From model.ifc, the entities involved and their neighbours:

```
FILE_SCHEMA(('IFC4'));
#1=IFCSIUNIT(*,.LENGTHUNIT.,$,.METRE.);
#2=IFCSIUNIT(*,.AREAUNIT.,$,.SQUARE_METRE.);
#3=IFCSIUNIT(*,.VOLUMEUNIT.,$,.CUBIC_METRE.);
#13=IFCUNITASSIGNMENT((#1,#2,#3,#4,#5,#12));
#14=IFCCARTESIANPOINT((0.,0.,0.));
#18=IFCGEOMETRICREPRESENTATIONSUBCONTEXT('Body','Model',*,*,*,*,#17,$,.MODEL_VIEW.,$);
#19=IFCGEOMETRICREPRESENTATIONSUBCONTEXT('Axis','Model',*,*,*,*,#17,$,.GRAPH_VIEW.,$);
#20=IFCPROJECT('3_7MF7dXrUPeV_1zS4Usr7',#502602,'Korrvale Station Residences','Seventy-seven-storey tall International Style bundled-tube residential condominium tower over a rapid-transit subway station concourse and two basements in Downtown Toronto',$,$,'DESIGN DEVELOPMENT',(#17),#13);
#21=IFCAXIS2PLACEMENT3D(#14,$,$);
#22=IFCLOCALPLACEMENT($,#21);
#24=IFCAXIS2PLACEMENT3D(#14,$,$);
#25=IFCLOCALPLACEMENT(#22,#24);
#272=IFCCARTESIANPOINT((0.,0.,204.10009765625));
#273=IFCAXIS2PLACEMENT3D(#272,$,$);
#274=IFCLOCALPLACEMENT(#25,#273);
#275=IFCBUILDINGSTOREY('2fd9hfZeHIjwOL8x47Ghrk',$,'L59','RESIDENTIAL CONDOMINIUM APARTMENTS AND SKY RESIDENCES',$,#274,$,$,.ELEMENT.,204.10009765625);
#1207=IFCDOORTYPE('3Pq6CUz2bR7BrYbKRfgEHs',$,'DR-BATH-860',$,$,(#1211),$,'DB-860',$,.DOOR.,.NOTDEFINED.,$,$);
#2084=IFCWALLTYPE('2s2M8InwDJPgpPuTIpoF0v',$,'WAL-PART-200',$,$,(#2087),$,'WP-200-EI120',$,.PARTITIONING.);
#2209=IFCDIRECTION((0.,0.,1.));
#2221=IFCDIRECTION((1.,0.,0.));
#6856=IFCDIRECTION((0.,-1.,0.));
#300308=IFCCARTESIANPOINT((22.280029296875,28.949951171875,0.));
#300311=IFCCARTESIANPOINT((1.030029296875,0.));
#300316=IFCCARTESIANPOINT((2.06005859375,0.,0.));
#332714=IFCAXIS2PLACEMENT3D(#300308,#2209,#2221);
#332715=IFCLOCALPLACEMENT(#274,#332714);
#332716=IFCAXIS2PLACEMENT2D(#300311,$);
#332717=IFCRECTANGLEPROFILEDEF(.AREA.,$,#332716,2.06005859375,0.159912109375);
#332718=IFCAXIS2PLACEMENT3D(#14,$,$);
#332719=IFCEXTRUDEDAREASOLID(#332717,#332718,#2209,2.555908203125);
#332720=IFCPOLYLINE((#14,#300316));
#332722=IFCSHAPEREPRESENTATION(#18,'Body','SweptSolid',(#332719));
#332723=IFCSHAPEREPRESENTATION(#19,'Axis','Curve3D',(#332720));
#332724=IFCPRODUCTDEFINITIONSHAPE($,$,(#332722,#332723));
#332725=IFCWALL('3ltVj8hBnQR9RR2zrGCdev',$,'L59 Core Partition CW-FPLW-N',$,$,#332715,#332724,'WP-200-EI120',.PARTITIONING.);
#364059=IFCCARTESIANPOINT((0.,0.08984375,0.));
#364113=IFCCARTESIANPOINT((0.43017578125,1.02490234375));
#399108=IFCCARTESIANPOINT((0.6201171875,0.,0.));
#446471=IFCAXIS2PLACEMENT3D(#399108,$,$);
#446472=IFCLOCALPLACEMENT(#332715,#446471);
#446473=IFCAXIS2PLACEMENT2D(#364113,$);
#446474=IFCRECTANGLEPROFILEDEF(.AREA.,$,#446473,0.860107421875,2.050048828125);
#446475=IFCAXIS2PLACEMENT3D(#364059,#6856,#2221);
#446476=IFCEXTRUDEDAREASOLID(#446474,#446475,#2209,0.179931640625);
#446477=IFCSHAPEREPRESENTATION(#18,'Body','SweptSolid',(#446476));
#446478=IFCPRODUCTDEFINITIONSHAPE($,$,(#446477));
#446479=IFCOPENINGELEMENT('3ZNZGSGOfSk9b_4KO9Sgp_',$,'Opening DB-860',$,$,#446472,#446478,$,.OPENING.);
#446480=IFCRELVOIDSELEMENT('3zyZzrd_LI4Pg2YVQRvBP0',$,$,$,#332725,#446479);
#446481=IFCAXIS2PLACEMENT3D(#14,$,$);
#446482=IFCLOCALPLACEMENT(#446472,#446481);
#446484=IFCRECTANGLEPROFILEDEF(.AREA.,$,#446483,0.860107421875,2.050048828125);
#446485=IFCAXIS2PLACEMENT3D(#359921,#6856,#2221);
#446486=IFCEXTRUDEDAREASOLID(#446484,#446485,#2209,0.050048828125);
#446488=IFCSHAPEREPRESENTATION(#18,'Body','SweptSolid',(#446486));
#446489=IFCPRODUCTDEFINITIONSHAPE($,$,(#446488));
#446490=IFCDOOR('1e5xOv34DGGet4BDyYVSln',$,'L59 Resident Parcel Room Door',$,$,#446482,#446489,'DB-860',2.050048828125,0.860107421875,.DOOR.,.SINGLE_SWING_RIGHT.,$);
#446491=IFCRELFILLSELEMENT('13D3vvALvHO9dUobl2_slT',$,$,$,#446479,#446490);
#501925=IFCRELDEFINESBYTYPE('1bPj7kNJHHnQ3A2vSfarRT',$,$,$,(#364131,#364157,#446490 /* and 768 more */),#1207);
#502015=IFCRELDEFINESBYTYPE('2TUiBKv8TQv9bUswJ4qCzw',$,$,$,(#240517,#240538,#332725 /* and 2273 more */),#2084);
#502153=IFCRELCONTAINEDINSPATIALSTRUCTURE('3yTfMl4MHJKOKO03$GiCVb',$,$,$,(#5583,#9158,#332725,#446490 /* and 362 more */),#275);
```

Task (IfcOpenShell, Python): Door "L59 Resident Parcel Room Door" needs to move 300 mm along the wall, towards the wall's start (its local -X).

```python
import ifcopenshell
import ifcopenshell.api.geometry
import ifcopenshell.util.placement

model = ifcopenshell.open("model.ifc")

door = model.by_guid("1e5xOv34DGGet4BDyYVSln")
opening = door.FillsVoids[0].RelatingOpeningElement
wall = opening.VoidsElements[0].RelatingBuildingElement

wall_matrix = ifcopenshell.util.placement.get_local_placement(wall.ObjectPlacement)
shift = wall_matrix[:3, 0] * -0.3
before = ifcopenshell.util.placement.get_local_placement(door.ObjectPlacement)[:3, 3].copy()

# The door is placed relative to its opening, so it follows when the opening moves.
matrix = ifcopenshell.util.placement.get_local_placement(opening.ObjectPlacement)
matrix[:3, 3] += shift
ifcopenshell.api.geometry.edit_object_placement(
    model, product=opening, matrix=matrix, is_si=False, should_transform_children=True
)

after = ifcopenshell.util.placement.get_local_placement(door.ObjectPlacement)[:3, 3]
print("door moved by", (after - before).round(3) + 0.0)

model.write("model_updated.ifc")
```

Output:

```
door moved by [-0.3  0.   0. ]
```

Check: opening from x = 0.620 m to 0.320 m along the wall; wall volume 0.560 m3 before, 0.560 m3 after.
